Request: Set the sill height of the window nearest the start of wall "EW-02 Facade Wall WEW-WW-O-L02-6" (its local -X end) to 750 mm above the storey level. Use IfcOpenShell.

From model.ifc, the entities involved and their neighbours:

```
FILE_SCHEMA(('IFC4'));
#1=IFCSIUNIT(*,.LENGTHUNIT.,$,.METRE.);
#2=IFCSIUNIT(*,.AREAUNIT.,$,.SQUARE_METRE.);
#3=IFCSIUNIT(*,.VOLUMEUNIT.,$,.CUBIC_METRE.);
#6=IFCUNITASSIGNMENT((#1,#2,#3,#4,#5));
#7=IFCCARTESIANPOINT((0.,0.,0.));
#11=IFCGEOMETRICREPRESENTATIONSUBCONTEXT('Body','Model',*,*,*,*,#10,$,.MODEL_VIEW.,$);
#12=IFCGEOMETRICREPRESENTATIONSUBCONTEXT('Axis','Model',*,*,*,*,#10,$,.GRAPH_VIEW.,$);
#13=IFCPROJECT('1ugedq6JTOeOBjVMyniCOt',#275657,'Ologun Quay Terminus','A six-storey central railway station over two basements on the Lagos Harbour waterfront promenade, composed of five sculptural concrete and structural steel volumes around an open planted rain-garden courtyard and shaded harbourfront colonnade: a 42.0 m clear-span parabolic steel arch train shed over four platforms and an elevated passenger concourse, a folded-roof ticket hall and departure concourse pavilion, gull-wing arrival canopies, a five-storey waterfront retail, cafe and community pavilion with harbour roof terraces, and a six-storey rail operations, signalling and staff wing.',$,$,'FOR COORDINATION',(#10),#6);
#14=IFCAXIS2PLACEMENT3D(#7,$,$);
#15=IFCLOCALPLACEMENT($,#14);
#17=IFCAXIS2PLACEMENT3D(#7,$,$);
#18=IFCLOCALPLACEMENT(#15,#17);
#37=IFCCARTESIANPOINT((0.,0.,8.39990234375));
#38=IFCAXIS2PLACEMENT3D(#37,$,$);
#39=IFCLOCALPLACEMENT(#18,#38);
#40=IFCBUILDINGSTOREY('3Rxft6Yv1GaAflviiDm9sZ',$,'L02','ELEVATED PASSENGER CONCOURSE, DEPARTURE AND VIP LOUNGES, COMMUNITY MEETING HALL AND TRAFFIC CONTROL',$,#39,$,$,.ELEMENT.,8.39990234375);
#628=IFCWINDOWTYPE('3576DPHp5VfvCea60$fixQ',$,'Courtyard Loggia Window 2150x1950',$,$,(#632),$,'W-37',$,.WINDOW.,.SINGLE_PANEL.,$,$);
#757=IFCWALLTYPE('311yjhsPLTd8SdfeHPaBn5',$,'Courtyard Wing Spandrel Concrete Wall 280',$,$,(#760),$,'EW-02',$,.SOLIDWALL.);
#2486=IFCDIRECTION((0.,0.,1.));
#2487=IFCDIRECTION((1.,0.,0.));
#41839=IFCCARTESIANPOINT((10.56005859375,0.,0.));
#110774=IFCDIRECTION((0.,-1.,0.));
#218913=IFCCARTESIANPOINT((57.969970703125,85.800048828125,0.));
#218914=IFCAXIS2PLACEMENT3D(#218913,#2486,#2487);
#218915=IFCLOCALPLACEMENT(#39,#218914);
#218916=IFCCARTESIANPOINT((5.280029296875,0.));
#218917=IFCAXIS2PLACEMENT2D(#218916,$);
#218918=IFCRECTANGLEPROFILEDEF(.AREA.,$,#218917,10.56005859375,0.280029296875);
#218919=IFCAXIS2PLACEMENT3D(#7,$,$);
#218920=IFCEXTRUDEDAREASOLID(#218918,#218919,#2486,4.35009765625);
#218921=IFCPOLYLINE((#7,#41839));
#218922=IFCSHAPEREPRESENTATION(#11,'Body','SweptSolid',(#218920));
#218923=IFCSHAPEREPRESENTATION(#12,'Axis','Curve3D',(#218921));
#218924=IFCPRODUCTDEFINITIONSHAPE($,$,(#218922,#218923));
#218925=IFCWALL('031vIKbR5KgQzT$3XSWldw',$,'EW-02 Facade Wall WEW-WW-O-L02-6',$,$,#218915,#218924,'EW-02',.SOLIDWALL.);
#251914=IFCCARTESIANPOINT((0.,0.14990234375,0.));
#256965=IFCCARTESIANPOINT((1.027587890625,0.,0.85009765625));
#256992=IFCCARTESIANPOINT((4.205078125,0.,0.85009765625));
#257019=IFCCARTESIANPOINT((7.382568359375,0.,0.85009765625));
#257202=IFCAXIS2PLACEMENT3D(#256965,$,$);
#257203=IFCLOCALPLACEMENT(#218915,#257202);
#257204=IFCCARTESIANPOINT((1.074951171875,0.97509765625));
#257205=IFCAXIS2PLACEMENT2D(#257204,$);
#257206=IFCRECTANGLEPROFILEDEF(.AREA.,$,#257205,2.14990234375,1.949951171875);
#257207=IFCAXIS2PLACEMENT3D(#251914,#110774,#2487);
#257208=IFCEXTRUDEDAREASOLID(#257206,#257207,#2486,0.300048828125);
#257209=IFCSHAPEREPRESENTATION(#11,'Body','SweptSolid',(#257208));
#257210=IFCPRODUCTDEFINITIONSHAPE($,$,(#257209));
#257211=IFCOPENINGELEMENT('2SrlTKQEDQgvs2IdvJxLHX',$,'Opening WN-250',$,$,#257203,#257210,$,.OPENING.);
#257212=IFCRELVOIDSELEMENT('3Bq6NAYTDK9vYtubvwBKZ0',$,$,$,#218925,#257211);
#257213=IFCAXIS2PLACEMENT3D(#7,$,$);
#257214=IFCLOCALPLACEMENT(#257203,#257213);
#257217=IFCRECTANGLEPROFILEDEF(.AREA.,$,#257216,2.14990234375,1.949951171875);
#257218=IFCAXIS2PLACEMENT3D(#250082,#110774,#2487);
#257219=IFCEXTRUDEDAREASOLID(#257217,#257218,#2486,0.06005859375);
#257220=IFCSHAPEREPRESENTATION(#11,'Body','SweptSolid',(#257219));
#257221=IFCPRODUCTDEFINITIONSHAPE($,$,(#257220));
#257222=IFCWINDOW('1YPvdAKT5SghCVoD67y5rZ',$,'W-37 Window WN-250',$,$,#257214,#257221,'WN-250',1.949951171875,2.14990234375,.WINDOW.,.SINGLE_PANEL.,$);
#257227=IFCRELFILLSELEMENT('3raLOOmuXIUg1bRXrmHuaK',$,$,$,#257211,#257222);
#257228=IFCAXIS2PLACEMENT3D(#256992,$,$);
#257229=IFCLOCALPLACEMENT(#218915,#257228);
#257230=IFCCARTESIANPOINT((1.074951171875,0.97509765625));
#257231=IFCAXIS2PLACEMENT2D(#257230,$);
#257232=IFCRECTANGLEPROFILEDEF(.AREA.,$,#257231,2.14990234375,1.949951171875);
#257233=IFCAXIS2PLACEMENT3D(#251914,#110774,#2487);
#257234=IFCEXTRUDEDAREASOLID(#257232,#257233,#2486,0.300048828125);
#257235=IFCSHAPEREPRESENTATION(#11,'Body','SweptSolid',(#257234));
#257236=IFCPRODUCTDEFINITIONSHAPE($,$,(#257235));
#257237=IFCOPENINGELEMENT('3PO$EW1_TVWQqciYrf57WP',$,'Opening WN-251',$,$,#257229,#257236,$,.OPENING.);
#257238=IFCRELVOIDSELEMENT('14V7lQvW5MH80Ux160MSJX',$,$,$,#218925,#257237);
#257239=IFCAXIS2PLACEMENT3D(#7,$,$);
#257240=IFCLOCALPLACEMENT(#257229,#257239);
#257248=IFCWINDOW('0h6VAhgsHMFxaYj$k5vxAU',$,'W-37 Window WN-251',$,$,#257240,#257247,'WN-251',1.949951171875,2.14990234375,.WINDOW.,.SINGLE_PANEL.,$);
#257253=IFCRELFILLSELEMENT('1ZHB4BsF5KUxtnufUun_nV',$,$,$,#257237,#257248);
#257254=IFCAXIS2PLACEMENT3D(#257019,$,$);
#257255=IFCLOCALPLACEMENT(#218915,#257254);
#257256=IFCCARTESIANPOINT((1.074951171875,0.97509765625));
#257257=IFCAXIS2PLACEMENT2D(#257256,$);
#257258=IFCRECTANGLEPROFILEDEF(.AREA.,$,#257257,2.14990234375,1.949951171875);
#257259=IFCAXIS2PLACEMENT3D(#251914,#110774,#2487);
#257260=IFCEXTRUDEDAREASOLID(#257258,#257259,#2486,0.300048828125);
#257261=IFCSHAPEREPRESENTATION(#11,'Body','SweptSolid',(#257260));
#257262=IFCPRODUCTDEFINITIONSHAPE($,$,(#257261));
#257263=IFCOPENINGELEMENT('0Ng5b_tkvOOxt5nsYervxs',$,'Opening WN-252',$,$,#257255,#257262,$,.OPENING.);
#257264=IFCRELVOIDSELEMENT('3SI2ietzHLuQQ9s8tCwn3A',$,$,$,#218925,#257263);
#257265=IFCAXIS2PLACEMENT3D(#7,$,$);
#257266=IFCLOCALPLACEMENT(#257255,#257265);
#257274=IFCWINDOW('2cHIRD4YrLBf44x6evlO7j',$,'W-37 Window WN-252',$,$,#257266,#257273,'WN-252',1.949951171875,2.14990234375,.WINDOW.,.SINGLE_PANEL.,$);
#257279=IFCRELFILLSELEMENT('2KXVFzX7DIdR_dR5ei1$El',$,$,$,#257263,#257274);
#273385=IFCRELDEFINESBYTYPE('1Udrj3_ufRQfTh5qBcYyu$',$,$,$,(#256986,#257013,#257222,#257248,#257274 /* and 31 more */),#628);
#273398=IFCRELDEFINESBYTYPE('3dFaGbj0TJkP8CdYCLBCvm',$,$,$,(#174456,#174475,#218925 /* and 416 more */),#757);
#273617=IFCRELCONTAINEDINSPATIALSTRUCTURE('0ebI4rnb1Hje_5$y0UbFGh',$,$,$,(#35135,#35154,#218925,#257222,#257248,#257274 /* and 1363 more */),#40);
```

```python
import numpy as np
import ifcopenshell
import ifcopenshell.api.geometry
import ifcopenshell.geom
import ifcopenshell.util.element
import ifcopenshell.util.placement
import ifcopenshell.util.shape
import ifcopenshell.util.unit

model = ifcopenshell.open("model.ifc")
unit_scale = ifcopenshell.util.unit.calculate_unit_scale(model)

window = model.by_id(257222)
opening = window.FillsVoids[0].RelatingOpeningElement
storey = ifcopenshell.util.element.get_container(window, ifc_class="IfcBuildingStorey")
level = ifcopenshell.util.placement.get_local_placement(storey.ObjectPlacement)[2, 3]

# The opening's origin need not be at the sill, so measure its lowest point.
shape = ifcopenshell.geom.create_shape(ifcopenshell.geom.settings(), opening)
bottom = ifcopenshell.util.shape.get_shape_bottom_elevation(shape, shape.geometry) / unit_scale
dz = level + 0.75 - bottom

shift = np.array([0.0, 0.0, dz])
# The window is placed relative to its opening, so it follows when the opening moves.
matrix = ifcopenshell.util.placement.get_local_placement(opening.ObjectPlacement)
matrix[:3, 3] += shift
ifcopenshell.api.geometry.edit_object_placement(
    model, product=opening, matrix=matrix, is_si=False, should_transform_children=True
)

print(f"moved by {dz * unit_scale:+.3f} m")

model.write("model_v2.ifc")
```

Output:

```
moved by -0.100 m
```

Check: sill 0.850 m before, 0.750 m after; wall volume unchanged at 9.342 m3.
